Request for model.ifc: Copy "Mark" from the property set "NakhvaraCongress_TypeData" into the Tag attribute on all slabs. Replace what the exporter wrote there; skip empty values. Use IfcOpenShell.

First a look at what the model holds.

```python
import ifcopenshell
import ifcopenshell.util.element

model = ifcopenshell.open("model.ifc")
print(model.schema)
slabs = model.by_type("IfcSlab")
print(len(slabs), "slabs")
for e in slabs[:8]:
    source = ifcopenshell.util.element.get_pset(e, "NakhvaraCongress_TypeData", "Mark")
    target = e.Tag
    print(e.id(), repr(source), repr(target), sep=" | ")
```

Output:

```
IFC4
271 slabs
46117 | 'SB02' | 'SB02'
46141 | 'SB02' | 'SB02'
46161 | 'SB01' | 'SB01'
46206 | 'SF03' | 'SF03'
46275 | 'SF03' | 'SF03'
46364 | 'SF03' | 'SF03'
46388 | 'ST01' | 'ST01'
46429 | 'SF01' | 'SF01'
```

```python
import ifcopenshell
import ifcopenshell.util.element

model = ifcopenshell.open("model.ifc")

count = 0
for e in model.by_type("IfcSlab"):
    value = ifcopenshell.util.element.get_pset(e, "NakhvaraCongress_TypeData", "Mark")
    current = e.Tag
    if not value or not value.strip() or current == value:
        continue
    e.Tag = value
    count += 1

print(count, "slabs updated")

model.write("model-out.ifc")
```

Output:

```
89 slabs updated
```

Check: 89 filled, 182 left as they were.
